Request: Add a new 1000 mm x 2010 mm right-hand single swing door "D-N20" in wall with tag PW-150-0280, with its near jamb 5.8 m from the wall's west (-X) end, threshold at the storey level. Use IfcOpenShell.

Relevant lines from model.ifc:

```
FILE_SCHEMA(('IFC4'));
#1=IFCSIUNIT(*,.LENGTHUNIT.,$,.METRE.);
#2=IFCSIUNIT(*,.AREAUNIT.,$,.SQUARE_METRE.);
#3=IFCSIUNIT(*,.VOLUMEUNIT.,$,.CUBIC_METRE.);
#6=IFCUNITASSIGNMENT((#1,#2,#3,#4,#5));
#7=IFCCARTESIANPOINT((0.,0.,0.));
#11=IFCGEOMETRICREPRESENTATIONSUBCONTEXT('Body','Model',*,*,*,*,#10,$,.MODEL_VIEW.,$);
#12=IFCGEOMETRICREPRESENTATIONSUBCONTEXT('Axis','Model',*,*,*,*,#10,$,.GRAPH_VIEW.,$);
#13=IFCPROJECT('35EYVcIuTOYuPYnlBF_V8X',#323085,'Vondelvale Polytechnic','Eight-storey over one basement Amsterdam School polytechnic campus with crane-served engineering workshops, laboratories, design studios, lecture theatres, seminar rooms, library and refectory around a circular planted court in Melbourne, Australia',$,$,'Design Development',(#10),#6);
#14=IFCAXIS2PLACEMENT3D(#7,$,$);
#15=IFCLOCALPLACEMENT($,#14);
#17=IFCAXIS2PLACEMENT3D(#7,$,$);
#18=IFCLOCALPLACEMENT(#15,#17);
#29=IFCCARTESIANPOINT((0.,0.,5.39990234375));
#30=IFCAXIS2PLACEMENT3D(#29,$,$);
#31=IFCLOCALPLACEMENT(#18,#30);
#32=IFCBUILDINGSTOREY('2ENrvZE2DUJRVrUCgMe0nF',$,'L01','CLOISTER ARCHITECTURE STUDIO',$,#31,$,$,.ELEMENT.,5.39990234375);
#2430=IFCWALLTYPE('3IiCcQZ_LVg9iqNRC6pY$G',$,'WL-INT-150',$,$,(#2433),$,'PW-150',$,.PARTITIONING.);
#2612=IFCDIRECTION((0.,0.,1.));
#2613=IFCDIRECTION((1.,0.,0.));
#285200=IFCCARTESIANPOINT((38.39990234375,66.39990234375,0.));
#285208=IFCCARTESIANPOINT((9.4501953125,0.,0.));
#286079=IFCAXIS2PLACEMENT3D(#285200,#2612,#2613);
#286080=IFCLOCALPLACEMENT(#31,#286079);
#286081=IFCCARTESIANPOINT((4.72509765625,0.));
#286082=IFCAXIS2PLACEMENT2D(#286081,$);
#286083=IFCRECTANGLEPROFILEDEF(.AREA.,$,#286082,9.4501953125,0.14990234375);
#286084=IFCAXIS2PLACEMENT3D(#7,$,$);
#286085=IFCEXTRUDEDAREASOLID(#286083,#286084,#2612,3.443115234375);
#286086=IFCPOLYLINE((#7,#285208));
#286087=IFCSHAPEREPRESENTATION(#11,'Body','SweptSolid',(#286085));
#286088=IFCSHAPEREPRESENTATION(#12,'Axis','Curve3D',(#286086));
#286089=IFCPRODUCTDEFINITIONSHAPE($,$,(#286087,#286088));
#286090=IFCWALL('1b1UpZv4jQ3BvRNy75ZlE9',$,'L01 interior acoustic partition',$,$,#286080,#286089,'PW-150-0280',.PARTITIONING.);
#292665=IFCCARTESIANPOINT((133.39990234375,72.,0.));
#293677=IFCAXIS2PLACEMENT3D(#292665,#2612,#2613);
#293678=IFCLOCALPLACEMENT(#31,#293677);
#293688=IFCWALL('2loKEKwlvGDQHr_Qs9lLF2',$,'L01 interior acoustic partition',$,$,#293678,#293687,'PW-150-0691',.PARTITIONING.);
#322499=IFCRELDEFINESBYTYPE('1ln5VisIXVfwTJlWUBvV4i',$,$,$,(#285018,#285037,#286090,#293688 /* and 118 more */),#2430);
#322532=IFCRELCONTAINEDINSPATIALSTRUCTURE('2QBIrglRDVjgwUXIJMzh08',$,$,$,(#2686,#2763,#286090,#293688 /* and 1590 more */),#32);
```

```python
import numpy as np
import ifcopenshell
import ifcopenshell.api.feature
import ifcopenshell.api.geometry
import ifcopenshell.api.root
import ifcopenshell.api.spatial
import ifcopenshell.geom
import ifcopenshell.util.element
import ifcopenshell.util.placement
import ifcopenshell.util.representation
import ifcopenshell.util.shape
import ifcopenshell.util.unit

model = ifcopenshell.open("model.ifc")
unit_scale = ifcopenshell.util.unit.calculate_unit_scale(model)
settings = ifcopenshell.geom.settings()


def volume(element):
    """Net volume in cubic metres, openings subtracted."""
    shape = ifcopenshell.geom.create_shape(settings, element)
    return ifcopenshell.util.shape.get_volume(shape.geometry)


wall = model.by_guid("1b1UpZv4jQ3BvRNy75ZlE9")
storey = ifcopenshell.util.element.get_container(wall, ifc_class="IfcBuildingStorey")
context = ifcopenshell.util.representation.get_context(model, "Model", "Body", "MODEL_VIEW")
before = volume(wall)

width, height, from_end, sill = 1, 2.01, 5.8, 0.0  # metres

# The wall runs along its own X axis, and the end named is its -X end.
wall_shape = ifcopenshell.geom.create_shape(settings, wall)
x, y, z = ifcopenshell.util.shape.get_vertices(wall_shape.geometry).T
start = x.min() + from_end
face, thickness = float(y.min()), float(y.max() - y.min())
wall_matrix = ifcopenshell.util.placement.get_local_placement(wall.ObjectPlacement)
level = ifcopenshell.util.placement.get_local_placement(storey.ObjectPlacement)[2, 3]


def in_wall(x, y):
    """Placement at x, y metres in the wall's axes, at sill height."""
    matrix = wall_matrix.copy()
    matrix[:, 3] = wall_matrix @ np.array([x / unit_scale, y / unit_scale, 0.0, 1.0])
    matrix[2, 3] = level + sill / unit_scale
    return matrix


# Opening: a box that overshoots both wall faces by 50 mm.
opening = ifcopenshell.api.root.create_entity(model, ifc_class="IfcOpeningElement", predefined_type="OPENING")
box = ifcopenshell.api.geometry.add_wall_representation(
    model, context=context, length=width, height=height, thickness=thickness + 0.1
)
ifcopenshell.api.geometry.assign_representation(model, product=opening, representation=box)
ifcopenshell.api.geometry.edit_object_placement(model, product=opening, matrix=in_wall(start, face - 0.05), is_si=False)
ifcopenshell.api.feature.add_feature(model, feature=opening, element=wall)

door = ifcopenshell.api.root.create_entity(model, ifc_class="IfcDoor", name="D-N20", predefined_type="DOOR")
door.OverallWidth, door.OverallHeight = width / unit_scale, height / unit_scale
door.OperationType = "SINGLE_SWING_RIGHT"
body = ifcopenshell.api.geometry.add_door_representation(
    model,
    context=context,
    overall_width=door.OverallWidth,
    overall_height=door.OverallHeight,
    operation_type="SINGLE_SWING_RIGHT",
    lining_properties={"LiningDepth": thickness / unit_scale, "ThresholdDepth": thickness / unit_scale},
)
ifcopenshell.api.geometry.assign_representation(model, product=door, representation=body)
ifcopenshell.api.spatial.assign_container(model, products=[door], relating_structure=storey)
ifcopenshell.api.feature.add_filling(model, opening=opening, element=door)

# The lining spans the wall, so the door starts at the wall face.
ifcopenshell.api.geometry.edit_object_placement(model, product=door, matrix=in_wall(start, face), is_si=False)

after = volume(wall)

print(f"wall volume {before:.3f} -> {after:.3f} m3")

model.write("model_edited.ifc")
```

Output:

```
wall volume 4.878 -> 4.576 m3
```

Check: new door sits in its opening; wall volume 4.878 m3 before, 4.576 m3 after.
